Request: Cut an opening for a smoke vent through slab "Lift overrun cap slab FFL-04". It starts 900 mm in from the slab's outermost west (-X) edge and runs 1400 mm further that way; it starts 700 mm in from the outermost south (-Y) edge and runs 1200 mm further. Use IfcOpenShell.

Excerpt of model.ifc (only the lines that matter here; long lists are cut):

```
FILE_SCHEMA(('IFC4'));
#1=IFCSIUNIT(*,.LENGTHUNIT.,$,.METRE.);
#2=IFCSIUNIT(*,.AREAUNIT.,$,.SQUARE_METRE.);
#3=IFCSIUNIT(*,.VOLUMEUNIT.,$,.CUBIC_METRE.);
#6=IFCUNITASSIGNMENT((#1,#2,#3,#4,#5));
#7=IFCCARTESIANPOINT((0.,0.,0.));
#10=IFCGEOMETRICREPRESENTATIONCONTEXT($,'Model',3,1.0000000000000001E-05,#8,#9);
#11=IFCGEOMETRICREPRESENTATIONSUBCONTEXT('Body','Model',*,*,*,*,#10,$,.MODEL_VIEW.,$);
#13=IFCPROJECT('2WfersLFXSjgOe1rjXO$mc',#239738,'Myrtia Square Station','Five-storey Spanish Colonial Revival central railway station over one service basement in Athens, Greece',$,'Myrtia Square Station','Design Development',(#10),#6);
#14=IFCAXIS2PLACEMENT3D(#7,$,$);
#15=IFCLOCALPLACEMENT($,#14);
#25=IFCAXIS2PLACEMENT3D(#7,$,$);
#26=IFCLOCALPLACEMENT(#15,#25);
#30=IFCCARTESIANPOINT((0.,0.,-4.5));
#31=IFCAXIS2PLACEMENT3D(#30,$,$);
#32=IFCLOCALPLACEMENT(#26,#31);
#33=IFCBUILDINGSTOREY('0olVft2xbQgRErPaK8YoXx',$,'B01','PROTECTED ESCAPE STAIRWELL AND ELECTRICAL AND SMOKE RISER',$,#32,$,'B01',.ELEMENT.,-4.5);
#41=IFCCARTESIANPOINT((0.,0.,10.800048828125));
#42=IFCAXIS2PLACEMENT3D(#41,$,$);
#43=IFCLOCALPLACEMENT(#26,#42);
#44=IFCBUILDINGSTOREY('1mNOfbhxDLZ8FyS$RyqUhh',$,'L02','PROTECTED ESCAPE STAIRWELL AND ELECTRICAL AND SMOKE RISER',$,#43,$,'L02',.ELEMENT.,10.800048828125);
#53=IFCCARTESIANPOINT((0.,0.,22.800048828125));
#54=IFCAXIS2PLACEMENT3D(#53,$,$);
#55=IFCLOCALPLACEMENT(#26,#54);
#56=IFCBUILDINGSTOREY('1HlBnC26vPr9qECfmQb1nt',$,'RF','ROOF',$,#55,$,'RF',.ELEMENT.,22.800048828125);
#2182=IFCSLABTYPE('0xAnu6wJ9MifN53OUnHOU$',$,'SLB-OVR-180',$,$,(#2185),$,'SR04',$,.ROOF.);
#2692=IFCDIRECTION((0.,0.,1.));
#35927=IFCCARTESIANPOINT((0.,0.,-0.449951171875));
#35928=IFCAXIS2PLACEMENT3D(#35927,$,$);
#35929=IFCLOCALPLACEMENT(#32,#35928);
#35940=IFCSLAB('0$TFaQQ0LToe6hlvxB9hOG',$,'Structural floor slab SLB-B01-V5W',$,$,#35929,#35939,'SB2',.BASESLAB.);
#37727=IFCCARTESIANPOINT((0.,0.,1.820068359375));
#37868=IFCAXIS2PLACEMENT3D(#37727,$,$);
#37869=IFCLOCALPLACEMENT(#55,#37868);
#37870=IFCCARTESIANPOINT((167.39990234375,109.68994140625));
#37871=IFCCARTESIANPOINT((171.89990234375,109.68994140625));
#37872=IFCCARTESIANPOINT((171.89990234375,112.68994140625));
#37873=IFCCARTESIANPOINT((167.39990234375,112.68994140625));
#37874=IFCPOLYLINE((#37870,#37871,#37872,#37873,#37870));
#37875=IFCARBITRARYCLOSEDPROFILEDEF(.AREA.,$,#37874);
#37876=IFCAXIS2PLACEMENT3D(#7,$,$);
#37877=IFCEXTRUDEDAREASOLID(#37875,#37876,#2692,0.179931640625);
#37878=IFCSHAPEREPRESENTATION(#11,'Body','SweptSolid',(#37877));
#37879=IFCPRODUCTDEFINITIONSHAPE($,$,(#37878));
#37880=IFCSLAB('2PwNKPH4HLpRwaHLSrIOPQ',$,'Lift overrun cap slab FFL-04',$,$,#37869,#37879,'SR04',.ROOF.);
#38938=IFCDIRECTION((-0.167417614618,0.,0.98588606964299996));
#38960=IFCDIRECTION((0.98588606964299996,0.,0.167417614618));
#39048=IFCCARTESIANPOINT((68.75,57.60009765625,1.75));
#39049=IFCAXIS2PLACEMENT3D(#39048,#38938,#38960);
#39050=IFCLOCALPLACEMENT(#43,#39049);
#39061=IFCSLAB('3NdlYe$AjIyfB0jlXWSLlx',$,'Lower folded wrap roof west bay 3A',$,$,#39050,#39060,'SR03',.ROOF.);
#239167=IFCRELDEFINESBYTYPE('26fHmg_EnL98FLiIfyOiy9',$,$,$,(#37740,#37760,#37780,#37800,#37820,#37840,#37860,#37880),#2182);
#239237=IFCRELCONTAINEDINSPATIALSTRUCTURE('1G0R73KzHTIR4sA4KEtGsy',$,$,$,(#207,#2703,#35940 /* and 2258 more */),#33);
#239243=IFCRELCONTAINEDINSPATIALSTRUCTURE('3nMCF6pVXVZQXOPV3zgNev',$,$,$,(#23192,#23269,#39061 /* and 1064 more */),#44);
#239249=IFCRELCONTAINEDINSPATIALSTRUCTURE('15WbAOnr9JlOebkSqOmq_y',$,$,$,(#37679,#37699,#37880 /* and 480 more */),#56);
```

```python
import numpy as np
import ifcopenshell
import ifcopenshell.api.feature
import ifcopenshell.api.geometry
import ifcopenshell.api.root
import ifcopenshell.geom
import ifcopenshell.util.placement
import ifcopenshell.util.representation
import ifcopenshell.util.shape
import ifcopenshell.util.unit

model = ifcopenshell.open("model.ifc")
unit_scale = ifcopenshell.util.unit.calculate_unit_scale(model)
settings = ifcopenshell.geom.settings()


def volume(element):
    """Net volume in cubic metres, openings subtracted."""
    shape = ifcopenshell.geom.create_shape(settings, element)
    return ifcopenshell.util.shape.get_volume(shape.geometry)


slab = model.by_id(37880)
before = volume(slab)

# Extent in the slab's own axes, in metres. The edges named are its -X and -Y sides.
slab_shape = ifcopenshell.geom.create_shape(settings, slab)
vertices = ifcopenshell.util.shape.get_vertices(slab_shape.geometry)
x_min, y_min, bottom = vertices.min(axis=0)
top = vertices[:, 2].max()

opening = ifcopenshell.api.root.create_entity(model, ifc_class="IfcOpeningElement", name="Smoke vent opening", predefined_type="OPENING")
context = ifcopenshell.util.representation.get_context(model, "Model", "Body", "MODEL_VIEW")
width, depth = 1.4, 1.2
outline = [(0.0, 0.0), (width, 0.0), (width, depth), (0.0, depth), (0.0, 0.0)]
# Overshoot both faces by 50 mm so the cut is clean.
shape = ifcopenshell.api.geometry.add_slab_representation(
    model, context=context, depth=top - bottom + 0.1, polyline=outline
)
ifcopenshell.api.geometry.assign_representation(model, product=opening, representation=shape)

matrix = ifcopenshell.util.placement.get_local_placement(slab.ObjectPlacement)
matrix[:, 3] = matrix @ np.append(np.array([x_min + 0.9, y_min + 0.7, bottom - 0.05]) / unit_scale, 1.0)
ifcopenshell.api.geometry.edit_object_placement(model, product=opening, matrix=matrix, is_si=False)
ifcopenshell.api.feature.add_feature(model, feature=opening, element=slab)

after = volume(slab)

print(f"slab volume {before:.3f} -> {after:.3f} m3")

model.write("model_rev.ifc")
```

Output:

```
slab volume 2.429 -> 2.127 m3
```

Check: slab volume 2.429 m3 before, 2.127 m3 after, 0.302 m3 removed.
